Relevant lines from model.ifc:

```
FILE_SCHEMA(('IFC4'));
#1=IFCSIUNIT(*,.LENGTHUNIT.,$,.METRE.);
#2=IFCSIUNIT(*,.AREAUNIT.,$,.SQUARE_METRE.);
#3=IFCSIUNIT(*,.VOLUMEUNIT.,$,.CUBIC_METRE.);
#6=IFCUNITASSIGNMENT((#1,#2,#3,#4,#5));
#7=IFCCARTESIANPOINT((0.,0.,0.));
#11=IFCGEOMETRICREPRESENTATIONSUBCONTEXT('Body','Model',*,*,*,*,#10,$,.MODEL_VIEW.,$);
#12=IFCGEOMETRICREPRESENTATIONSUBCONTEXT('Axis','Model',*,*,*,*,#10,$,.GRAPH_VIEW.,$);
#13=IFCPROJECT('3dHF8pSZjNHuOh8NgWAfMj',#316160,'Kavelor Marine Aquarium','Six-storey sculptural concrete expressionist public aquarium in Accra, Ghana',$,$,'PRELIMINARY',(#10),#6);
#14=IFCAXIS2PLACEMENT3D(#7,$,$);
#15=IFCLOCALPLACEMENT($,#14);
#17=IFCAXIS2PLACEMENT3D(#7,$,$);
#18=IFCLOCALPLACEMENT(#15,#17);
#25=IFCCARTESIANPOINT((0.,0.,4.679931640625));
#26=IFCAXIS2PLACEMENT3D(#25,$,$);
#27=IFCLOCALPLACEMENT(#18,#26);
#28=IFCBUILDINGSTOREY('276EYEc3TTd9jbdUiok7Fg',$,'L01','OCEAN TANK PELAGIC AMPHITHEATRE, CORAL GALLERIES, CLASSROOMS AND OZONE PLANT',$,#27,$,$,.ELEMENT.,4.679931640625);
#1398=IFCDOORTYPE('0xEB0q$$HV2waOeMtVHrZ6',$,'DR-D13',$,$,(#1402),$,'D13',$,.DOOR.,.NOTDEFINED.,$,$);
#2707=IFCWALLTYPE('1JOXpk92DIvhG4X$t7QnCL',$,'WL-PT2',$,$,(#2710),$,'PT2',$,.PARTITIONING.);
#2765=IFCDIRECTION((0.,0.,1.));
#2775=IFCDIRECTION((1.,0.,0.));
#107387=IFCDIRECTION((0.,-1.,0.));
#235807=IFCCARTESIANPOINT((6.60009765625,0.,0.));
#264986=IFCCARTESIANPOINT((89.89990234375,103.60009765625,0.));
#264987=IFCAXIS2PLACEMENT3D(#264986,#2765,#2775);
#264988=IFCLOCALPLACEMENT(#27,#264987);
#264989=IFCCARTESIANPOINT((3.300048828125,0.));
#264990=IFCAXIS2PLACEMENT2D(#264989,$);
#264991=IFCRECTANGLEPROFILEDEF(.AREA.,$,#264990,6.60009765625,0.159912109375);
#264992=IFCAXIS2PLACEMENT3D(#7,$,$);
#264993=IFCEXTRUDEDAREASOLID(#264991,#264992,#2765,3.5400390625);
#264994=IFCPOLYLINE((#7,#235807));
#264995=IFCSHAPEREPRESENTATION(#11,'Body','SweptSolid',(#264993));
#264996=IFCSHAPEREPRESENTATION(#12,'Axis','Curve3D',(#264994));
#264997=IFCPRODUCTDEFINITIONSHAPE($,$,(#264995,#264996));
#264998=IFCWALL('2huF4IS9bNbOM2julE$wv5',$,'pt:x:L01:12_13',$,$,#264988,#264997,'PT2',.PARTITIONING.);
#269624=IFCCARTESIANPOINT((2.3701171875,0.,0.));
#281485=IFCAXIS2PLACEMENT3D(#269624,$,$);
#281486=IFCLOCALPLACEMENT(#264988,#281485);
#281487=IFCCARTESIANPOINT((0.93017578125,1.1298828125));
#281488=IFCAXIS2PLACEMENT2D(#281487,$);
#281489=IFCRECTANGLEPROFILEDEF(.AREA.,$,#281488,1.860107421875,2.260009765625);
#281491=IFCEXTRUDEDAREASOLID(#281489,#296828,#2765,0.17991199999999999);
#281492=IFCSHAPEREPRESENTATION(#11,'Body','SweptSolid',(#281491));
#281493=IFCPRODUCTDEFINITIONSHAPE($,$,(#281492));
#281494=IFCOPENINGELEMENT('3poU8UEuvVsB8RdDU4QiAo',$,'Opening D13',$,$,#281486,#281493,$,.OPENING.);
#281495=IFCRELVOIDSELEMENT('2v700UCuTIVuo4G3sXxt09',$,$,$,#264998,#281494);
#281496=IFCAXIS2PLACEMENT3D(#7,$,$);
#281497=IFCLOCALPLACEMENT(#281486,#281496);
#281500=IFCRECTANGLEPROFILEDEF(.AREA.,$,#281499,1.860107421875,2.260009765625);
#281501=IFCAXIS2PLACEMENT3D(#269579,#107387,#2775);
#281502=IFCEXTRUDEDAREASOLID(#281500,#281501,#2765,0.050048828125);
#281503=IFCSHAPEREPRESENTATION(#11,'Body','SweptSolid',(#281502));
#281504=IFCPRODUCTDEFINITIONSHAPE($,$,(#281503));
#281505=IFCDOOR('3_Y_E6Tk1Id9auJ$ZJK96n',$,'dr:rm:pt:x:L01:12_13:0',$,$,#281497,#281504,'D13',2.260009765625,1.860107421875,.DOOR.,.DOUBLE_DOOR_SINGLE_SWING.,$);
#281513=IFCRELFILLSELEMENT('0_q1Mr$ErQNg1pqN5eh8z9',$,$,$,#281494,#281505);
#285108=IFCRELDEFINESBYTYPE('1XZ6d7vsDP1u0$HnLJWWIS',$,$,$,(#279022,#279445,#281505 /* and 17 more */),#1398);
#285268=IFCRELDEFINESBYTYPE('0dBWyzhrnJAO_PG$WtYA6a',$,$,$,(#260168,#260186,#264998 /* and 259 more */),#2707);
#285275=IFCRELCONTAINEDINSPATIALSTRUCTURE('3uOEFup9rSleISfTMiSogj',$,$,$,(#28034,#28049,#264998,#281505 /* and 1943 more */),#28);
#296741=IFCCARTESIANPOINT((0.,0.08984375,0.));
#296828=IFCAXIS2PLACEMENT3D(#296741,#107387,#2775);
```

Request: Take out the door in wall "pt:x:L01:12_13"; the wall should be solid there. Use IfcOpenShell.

```python
import ifcopenshell
import ifcopenshell.api.feature
import ifcopenshell.api.root
import ifcopenshell.geom
import ifcopenshell.util.shape

model = ifcopenshell.open("model.ifc")
settings = ifcopenshell.geom.settings()


def volume(element):
    """Net volume in cubic metres, openings subtracted."""
    shape = ifcopenshell.geom.create_shape(settings, element)
    return ifcopenshell.util.shape.get_volume(shape.geometry)


door = model.by_id(281505)
opening = door.FillsVoids[0].RelatingOpeningElement
wall = opening.VoidsElements[0].RelatingBuildingElement
before = volume(wall)

ifcopenshell.api.root.remove_product(model, product=door)
ifcopenshell.api.feature.remove_feature(model, feature=opening)

after = volume(wall)

print(f"wall volume {before:.3f} -> {after:.3f} m3")

model.write("model_rev.ifc")
```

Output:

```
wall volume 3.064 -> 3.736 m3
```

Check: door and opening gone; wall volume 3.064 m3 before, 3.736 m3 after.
